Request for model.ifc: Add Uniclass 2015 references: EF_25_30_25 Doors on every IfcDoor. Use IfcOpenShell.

First a look at what the model holds.

```python
import ifcopenshell

model = ifcopenshell.open("model.ifc")
print(model.schema)
print("classifications:", [c.Name for c in model.by_type("IfcClassification")])
for ifc_class in ("IfcDoor", "IfcRoof", "IfcStair", "IfcWall", "IfcWindow"):
    print(ifc_class, len(model.by_type(ifc_class)))
```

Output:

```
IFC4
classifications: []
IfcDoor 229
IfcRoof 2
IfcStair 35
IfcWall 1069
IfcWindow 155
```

```python
import ifcopenshell
import ifcopenshell.api.classification

model = ifcopenshell.open("model.ifc")

system = ifcopenshell.api.classification.add_classification(model, classification="Uniclass 2015")

codes = {
    "IfcDoor": ("EF_25_30_25", "Doors"),
}
for ifc_class, (code, name) in codes.items():
    products = model.by_type(ifc_class)
    ifcopenshell.api.classification.add_reference(
        model, products=products, classification=system, identification=code, name=name
    )
    print(code, len(products))

model.write("model_updated.ifc")
```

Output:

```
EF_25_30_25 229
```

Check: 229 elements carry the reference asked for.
